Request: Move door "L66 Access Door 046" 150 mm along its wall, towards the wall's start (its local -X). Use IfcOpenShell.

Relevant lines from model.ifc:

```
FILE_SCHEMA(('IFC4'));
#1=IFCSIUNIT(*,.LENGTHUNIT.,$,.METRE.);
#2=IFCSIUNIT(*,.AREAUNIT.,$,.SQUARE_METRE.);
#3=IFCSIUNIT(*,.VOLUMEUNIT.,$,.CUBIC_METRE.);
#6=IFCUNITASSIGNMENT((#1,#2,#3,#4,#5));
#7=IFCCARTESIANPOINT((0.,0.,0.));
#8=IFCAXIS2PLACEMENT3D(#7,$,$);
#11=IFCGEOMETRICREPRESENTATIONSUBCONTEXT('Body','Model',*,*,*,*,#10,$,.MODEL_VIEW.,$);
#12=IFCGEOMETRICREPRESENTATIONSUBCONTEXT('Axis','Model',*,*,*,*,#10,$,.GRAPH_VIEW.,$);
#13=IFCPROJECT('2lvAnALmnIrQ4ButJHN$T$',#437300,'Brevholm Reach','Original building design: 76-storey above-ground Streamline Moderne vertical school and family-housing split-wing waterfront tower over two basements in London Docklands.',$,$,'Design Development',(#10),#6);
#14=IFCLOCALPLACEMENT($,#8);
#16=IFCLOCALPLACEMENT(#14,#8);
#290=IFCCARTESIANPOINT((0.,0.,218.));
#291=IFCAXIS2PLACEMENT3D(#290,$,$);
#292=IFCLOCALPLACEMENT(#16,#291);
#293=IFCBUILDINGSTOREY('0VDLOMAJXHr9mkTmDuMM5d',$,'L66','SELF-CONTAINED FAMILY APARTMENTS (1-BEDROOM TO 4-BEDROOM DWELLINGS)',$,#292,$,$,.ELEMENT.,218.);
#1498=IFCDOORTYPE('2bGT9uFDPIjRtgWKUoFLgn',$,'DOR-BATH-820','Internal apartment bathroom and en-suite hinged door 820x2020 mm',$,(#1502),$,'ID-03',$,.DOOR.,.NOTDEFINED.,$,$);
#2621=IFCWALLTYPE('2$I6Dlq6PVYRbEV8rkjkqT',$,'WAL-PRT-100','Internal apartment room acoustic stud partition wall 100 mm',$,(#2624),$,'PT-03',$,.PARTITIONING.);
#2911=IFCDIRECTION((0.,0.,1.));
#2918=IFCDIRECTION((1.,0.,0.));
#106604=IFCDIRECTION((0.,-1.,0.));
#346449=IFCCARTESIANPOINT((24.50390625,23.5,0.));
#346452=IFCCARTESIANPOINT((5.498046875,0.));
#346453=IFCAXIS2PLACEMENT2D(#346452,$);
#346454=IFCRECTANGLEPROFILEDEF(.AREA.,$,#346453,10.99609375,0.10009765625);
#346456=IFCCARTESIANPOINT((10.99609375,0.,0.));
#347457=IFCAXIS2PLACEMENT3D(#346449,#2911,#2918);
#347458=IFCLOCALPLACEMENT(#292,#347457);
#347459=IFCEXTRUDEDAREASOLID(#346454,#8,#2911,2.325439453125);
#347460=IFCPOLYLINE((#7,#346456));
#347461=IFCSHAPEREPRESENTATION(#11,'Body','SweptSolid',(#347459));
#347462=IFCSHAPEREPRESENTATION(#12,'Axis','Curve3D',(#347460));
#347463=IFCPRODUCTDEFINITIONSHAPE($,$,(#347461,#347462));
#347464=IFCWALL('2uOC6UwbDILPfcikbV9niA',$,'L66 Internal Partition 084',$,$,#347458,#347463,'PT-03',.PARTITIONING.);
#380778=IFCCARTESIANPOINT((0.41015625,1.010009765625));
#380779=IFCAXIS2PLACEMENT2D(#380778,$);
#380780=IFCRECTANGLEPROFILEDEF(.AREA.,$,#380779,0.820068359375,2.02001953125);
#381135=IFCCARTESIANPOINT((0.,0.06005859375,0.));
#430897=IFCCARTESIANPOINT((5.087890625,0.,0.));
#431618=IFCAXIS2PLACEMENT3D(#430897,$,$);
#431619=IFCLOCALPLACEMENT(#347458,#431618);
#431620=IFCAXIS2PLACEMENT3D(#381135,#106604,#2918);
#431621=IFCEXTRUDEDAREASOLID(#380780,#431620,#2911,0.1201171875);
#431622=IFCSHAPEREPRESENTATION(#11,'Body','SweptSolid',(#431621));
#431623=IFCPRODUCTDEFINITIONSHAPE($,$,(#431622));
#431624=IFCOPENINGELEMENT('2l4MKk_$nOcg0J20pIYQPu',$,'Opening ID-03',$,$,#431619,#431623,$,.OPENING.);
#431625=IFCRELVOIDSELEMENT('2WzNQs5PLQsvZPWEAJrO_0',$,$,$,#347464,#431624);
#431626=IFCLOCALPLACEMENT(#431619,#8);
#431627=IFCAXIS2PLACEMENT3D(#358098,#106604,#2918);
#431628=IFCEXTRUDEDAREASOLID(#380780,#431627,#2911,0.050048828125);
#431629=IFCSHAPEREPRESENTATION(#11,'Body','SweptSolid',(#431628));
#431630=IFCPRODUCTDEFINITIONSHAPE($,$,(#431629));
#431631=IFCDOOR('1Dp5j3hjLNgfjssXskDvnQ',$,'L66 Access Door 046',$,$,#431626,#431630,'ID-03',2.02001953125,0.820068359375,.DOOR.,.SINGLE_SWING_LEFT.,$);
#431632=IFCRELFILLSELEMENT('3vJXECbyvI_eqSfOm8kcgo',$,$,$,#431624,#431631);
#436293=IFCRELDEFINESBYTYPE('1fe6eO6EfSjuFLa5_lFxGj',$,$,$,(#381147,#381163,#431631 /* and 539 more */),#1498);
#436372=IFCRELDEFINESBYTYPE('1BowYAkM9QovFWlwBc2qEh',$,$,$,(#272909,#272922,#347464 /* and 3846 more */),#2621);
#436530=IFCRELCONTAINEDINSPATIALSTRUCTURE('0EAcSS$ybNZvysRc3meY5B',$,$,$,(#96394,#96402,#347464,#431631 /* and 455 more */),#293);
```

```python
import ifcopenshell
import ifcopenshell.api.geometry
import ifcopenshell.util.placement

model = ifcopenshell.open("model.ifc")

door = model.by_guid("1Dp5j3hjLNgfjssXskDvnQ")
opening = door.FillsVoids[0].RelatingOpeningElement
wall = opening.VoidsElements[0].RelatingBuildingElement

wall_matrix = ifcopenshell.util.placement.get_local_placement(wall.ObjectPlacement)
shift = wall_matrix[:3, 0] * -0.15
before = ifcopenshell.util.placement.get_local_placement(door.ObjectPlacement)[:3, 3].copy()

# The door is placed relative to its opening, so it follows when the opening moves.
matrix = ifcopenshell.util.placement.get_local_placement(opening.ObjectPlacement)
matrix[:3, 3] += shift
ifcopenshell.api.geometry.edit_object_placement(
    model, product=opening, matrix=matrix, is_si=False, should_transform_children=True
)

after = ifcopenshell.util.placement.get_local_placement(door.ObjectPlacement)[:3, 3]
print("door moved by", (after - before).round(3) + 0.0)

model.write("model_v2.ifc")
```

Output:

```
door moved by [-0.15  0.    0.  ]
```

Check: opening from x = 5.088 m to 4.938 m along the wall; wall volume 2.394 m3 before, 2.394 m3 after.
